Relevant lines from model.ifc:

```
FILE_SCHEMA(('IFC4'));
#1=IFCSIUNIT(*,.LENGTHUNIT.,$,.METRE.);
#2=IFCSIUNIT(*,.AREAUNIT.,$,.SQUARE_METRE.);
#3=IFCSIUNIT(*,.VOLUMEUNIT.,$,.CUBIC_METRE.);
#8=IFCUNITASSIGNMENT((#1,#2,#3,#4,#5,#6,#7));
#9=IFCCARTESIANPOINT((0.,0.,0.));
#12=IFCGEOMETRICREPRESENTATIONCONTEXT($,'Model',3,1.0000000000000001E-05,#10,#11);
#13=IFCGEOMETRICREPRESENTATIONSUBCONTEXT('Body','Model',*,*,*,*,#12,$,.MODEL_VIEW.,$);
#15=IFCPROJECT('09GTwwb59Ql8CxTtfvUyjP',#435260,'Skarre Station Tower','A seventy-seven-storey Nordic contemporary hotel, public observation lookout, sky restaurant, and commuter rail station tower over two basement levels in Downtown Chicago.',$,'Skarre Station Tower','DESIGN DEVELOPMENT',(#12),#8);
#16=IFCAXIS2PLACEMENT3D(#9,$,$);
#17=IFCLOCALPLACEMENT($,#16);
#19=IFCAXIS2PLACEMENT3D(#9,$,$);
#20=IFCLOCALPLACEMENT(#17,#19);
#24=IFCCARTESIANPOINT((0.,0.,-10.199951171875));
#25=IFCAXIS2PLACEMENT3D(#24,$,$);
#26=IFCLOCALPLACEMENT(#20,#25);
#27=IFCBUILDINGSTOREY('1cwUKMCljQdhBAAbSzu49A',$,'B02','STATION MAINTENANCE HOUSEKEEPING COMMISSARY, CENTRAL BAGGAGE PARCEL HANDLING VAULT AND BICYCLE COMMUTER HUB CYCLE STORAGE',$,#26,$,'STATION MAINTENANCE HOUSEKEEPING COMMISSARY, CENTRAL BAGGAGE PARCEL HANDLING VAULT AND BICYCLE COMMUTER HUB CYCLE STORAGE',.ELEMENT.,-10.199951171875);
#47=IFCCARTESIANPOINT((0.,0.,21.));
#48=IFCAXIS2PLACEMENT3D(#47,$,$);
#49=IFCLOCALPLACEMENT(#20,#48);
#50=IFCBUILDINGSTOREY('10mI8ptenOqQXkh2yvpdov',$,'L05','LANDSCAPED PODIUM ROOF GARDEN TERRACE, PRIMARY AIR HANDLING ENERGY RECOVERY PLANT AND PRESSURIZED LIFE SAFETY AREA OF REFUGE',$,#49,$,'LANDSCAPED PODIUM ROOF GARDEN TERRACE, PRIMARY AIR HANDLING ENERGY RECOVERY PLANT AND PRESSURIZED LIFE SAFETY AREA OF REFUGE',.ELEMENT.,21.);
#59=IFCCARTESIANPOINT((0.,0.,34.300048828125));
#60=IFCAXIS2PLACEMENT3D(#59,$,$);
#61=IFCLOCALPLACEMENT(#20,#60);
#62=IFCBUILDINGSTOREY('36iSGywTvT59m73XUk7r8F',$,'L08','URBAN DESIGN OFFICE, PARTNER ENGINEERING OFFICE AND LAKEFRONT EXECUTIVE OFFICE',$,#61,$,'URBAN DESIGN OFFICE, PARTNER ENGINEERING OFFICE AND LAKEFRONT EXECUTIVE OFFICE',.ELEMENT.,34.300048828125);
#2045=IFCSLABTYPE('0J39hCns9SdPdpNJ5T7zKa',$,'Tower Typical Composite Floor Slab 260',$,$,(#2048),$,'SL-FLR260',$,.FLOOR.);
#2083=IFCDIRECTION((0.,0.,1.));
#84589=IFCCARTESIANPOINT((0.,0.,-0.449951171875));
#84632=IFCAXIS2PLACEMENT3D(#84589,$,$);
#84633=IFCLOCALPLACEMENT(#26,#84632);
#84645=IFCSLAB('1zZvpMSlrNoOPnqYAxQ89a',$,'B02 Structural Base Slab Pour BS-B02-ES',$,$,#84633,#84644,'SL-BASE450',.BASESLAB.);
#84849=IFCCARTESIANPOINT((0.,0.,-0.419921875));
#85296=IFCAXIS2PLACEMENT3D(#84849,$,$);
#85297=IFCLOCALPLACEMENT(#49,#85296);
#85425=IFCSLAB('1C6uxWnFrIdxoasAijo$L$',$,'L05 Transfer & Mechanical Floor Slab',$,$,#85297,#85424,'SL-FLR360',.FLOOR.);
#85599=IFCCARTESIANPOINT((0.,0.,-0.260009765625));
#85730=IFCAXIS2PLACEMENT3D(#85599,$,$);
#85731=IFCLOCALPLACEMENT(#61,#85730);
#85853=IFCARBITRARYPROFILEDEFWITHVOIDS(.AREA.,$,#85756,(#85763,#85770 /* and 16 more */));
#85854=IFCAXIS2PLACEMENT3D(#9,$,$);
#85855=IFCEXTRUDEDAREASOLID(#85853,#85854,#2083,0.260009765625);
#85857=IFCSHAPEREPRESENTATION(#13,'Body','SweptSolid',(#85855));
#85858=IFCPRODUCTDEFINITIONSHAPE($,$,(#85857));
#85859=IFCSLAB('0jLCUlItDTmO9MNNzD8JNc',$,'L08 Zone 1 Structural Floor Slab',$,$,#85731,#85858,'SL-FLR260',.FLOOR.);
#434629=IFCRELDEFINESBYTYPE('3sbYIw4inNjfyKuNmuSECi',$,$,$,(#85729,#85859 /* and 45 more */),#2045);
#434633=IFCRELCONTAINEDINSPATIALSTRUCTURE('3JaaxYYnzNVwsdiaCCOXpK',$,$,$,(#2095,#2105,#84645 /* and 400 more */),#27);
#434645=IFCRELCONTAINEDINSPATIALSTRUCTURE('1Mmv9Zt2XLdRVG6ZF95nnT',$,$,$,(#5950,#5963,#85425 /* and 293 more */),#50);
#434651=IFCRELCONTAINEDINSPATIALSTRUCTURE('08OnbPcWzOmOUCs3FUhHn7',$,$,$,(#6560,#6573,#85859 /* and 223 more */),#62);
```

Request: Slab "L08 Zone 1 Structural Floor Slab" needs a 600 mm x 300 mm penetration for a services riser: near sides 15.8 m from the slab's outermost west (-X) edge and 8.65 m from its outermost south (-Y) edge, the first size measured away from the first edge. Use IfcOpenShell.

```python
import numpy as np
import ifcopenshell
import ifcopenshell.api.feature
import ifcopenshell.api.geometry
import ifcopenshell.api.root
import ifcopenshell.geom
import ifcopenshell.util.placement
import ifcopenshell.util.representation
import ifcopenshell.util.shape
import ifcopenshell.util.unit

model = ifcopenshell.open("model.ifc")
unit_scale = ifcopenshell.util.unit.calculate_unit_scale(model)
settings = ifcopenshell.geom.settings()


def volume(element):
    """Net volume in cubic metres, openings subtracted."""
    shape = ifcopenshell.geom.create_shape(settings, element)
    return ifcopenshell.util.shape.get_volume(shape.geometry)


slab = model.by_guid("0jLCUlItDTmO9MNNzD8JNc")
before = volume(slab)

# Extent in the slab's own axes, in metres. The edges named are its -X and -Y sides.
slab_shape = ifcopenshell.geom.create_shape(settings, slab)
vertices = ifcopenshell.util.shape.get_vertices(slab_shape.geometry)
x_min, y_min, bottom = vertices.min(axis=0)
top = vertices[:, 2].max()

opening = ifcopenshell.api.root.create_entity(model, ifc_class="IfcOpeningElement", name="Services riser opening", predefined_type="OPENING")
context = ifcopenshell.util.representation.get_context(model, "Model", "Body", "MODEL_VIEW")
width, depth = 0.6, 0.3
outline = [(0.0, 0.0), (width, 0.0), (width, depth), (0.0, depth), (0.0, 0.0)]
# Overshoot both faces by 50 mm so the cut is clean.
shape = ifcopenshell.api.geometry.add_slab_representation(
    model, context=context, depth=top - bottom + 0.1, polyline=outline
)
ifcopenshell.api.geometry.assign_representation(model, product=opening, representation=shape)

matrix = ifcopenshell.util.placement.get_local_placement(slab.ObjectPlacement)
matrix[:, 3] = matrix @ np.append(np.array([x_min + 15.8, y_min + 8.65, bottom - 0.05]) / unit_scale, 1.0)
ifcopenshell.api.geometry.edit_object_placement(model, product=opening, matrix=matrix, is_si=False)
ifcopenshell.api.feature.add_feature(model, feature=opening, element=slab)

after = volume(slab)

print(f"slab volume {before:.3f} -> {after:.3f} m3")

model.write("model_updated.ifc")
```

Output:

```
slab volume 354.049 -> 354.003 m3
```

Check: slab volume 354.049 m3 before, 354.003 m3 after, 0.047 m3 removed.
